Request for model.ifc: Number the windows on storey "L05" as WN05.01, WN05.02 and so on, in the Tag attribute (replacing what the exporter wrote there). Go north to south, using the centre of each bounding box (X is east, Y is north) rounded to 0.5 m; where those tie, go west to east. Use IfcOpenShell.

First a look at what the model holds.

```python
import ifcopenshell
import ifcopenshell.util.element
import ifcopenshell.util.placement

model = ifcopenshell.open("model.ifc")
print(model.schema)
storey = next(s for s in model.by_type("IfcBuildingStorey") if s.Name == "L05")
windows = [e for e in ifcopenshell.util.element.get_decomposition(storey) if e.is_a("IfcWindow")]
for e in sorted(windows, key=lambda e: e.id()):
    origin = ifcopenshell.util.placement.get_local_placement(e.ObjectPlacement)[:3, 3]
    print(e.id(), e.Tag, e.Name, origin.round(2) + 0.0, sep=" | ")
```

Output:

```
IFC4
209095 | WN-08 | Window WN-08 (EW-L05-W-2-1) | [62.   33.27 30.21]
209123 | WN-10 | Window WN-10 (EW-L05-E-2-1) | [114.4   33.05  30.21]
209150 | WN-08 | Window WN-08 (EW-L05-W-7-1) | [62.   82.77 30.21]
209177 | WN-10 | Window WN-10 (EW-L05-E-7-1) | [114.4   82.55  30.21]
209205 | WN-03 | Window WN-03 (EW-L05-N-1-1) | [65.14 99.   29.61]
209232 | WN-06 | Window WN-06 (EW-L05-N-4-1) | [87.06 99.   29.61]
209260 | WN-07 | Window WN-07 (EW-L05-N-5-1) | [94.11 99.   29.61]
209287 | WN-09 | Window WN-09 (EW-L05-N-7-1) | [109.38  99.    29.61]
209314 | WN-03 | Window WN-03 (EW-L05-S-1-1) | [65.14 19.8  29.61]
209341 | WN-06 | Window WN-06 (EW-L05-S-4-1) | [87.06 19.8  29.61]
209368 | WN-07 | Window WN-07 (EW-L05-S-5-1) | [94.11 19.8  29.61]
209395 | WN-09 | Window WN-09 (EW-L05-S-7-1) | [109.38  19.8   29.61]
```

```python
import ifcopenshell
import ifcopenshell.geom
import ifcopenshell.util.element
import ifcopenshell.util.shape

model = ifcopenshell.open("model.ifc")
settings = ifcopenshell.geom.settings()
settings.set("use-world-coords", True)


def centre(element):
    shape = ifcopenshell.geom.create_shape(settings, element)
    return ifcopenshell.util.shape.get_bbox_centroid(shape.geometry)


storey = next(s for s in model.by_type("IfcBuildingStorey") if s.Name == "L05")
windows = [e for e in ifcopenshell.util.element.get_decomposition(storey) if e.is_a("IfcWindow")]

# Insertion points can sit at a corner or the storey origin, so sort by the geometry (in metres).
centres = {e: centre(e) for e in windows}
windows.sort(key=lambda e: (-round(centres[e][1] / 0.5), centres[e][0]))

for i, e in enumerate(windows, start=1):
    number = f"WN05.{i:02d}"
    e.Tag = number
    print(e.id(), number)

model.write("model_updated.ifc")
```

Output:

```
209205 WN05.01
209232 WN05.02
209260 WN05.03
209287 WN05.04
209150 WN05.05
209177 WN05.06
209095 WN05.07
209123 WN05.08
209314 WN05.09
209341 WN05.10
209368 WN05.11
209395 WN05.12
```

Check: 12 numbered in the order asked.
